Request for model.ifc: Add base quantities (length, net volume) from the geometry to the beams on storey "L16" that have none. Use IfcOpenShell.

First a look at what the model holds.

```python
import ifcopenshell
import ifcopenshell.util.element
import ifcopenshell.util.unit

model = ifcopenshell.open("model.ifc")
print(model.schema)
for unit_type in ("LENGTHUNIT", "AREAUNIT", "VOLUMEUNIT"):
    print(unit_type, ifcopenshell.util.unit.calculate_unit_scale(model, unit_type))
storey = next(s for s in model.by_type("IfcBuildingStorey") if s.Name == "L16")
beams = [e for e in ifcopenshell.util.element.get_decomposition(storey) if e.is_a("IfcBeam")]
for e in sorted(beams, key=lambda e: e.id()):
    print(e.id(), e.is_a(), e.Name, list(ifcopenshell.util.element.get_psets(e, qtos_only=True)), sep=" | ")
```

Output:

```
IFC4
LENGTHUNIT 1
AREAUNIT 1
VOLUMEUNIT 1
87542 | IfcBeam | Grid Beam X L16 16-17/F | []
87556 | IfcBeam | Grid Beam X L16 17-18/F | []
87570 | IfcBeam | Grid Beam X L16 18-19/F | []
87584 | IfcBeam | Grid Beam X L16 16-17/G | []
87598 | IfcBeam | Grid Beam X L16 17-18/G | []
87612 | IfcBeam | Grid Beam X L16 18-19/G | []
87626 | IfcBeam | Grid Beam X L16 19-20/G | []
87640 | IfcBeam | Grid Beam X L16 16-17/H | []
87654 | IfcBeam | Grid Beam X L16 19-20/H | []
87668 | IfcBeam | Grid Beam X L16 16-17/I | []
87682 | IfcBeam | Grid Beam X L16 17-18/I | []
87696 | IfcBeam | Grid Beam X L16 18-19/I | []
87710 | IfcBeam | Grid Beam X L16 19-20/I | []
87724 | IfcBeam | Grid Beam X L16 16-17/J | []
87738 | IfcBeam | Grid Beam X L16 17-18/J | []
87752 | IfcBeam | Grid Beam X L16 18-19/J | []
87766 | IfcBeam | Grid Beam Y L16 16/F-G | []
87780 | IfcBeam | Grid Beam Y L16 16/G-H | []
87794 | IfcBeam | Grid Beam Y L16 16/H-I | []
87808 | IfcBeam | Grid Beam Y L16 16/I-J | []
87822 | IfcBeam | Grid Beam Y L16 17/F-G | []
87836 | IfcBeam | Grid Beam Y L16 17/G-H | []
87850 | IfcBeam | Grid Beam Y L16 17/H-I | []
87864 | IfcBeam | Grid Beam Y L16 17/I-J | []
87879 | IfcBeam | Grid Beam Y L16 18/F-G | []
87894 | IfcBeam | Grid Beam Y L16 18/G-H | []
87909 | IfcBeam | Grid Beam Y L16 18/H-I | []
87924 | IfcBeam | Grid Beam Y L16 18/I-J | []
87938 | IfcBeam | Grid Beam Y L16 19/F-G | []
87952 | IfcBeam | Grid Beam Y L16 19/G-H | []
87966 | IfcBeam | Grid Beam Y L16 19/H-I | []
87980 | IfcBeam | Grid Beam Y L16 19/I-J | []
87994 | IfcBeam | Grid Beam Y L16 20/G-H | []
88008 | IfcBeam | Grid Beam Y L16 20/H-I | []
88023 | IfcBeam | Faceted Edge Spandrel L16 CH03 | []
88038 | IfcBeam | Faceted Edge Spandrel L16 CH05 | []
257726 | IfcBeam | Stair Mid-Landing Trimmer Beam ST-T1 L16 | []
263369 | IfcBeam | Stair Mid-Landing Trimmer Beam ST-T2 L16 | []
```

```python
import ifcopenshell
import ifcopenshell.api.pset
import ifcopenshell.geom
import ifcopenshell.util.element
import ifcopenshell.util.shape
import ifcopenshell.util.unit

model = ifcopenshell.open("model.ifc")
unit_scale = ifcopenshell.util.unit.calculate_unit_scale(model)
volume_scale = ifcopenshell.util.unit.calculate_unit_scale(model, "VOLUMEUNIT")
settings = ifcopenshell.geom.settings()

storey = next(s for s in model.by_type("IfcBuildingStorey") if s.Name == "L16")
beams = [e for e in ifcopenshell.util.element.get_decomposition(storey) if e.is_a("IfcBeam")]

for e in sorted(beams, key=lambda e: e.id()):
    if ifcopenshell.util.element.get_psets(e, qtos_only=True, should_inherit=False):
        continue
    # Geometry comes back in metres, in the element's own axes.
    shape = ifcopenshell.geom.create_shape(settings, e)
    values = {
        "Length": ifcopenshell.util.shape.get_max_xyz(shape.geometry) / unit_scale,
        "NetVolume": ifcopenshell.util.shape.get_volume(shape.geometry) / volume_scale,
    }
    qto = ifcopenshell.api.pset.add_qto(model, product=e, name="Qto_BeamBaseQuantities")
    ifcopenshell.api.pset.edit_qto(model, qto=qto, properties=values)
    print(e.id(), {k: round(v, 3) for k, v in values.items()})

model.write("model_v2.ifc")
```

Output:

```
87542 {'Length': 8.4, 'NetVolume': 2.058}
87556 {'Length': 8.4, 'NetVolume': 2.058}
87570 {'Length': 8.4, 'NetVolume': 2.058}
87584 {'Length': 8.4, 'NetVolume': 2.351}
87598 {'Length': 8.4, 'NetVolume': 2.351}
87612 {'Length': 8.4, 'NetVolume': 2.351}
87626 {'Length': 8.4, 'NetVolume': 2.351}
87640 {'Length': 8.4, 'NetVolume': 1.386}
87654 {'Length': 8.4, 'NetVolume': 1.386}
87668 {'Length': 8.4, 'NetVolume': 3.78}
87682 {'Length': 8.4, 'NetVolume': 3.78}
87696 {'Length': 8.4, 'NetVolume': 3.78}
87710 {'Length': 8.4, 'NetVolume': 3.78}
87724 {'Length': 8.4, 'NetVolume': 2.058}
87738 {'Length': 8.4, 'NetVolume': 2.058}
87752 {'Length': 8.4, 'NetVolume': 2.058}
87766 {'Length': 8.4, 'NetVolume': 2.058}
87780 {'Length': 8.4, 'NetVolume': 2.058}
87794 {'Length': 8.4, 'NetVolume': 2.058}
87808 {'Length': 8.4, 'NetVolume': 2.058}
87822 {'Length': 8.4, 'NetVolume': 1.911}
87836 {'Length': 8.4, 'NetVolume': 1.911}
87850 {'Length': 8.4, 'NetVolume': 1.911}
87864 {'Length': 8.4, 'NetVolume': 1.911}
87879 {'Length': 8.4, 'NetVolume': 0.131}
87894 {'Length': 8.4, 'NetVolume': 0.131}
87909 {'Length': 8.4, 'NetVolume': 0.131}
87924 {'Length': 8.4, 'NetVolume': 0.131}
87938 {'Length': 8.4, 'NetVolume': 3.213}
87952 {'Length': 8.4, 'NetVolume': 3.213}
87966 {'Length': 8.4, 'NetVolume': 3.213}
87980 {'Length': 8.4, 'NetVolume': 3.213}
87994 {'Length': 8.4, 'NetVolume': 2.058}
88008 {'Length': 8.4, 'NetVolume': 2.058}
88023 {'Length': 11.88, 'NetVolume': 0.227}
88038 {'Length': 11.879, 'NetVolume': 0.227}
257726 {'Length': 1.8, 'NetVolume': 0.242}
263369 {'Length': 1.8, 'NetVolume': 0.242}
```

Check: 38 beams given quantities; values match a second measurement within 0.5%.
